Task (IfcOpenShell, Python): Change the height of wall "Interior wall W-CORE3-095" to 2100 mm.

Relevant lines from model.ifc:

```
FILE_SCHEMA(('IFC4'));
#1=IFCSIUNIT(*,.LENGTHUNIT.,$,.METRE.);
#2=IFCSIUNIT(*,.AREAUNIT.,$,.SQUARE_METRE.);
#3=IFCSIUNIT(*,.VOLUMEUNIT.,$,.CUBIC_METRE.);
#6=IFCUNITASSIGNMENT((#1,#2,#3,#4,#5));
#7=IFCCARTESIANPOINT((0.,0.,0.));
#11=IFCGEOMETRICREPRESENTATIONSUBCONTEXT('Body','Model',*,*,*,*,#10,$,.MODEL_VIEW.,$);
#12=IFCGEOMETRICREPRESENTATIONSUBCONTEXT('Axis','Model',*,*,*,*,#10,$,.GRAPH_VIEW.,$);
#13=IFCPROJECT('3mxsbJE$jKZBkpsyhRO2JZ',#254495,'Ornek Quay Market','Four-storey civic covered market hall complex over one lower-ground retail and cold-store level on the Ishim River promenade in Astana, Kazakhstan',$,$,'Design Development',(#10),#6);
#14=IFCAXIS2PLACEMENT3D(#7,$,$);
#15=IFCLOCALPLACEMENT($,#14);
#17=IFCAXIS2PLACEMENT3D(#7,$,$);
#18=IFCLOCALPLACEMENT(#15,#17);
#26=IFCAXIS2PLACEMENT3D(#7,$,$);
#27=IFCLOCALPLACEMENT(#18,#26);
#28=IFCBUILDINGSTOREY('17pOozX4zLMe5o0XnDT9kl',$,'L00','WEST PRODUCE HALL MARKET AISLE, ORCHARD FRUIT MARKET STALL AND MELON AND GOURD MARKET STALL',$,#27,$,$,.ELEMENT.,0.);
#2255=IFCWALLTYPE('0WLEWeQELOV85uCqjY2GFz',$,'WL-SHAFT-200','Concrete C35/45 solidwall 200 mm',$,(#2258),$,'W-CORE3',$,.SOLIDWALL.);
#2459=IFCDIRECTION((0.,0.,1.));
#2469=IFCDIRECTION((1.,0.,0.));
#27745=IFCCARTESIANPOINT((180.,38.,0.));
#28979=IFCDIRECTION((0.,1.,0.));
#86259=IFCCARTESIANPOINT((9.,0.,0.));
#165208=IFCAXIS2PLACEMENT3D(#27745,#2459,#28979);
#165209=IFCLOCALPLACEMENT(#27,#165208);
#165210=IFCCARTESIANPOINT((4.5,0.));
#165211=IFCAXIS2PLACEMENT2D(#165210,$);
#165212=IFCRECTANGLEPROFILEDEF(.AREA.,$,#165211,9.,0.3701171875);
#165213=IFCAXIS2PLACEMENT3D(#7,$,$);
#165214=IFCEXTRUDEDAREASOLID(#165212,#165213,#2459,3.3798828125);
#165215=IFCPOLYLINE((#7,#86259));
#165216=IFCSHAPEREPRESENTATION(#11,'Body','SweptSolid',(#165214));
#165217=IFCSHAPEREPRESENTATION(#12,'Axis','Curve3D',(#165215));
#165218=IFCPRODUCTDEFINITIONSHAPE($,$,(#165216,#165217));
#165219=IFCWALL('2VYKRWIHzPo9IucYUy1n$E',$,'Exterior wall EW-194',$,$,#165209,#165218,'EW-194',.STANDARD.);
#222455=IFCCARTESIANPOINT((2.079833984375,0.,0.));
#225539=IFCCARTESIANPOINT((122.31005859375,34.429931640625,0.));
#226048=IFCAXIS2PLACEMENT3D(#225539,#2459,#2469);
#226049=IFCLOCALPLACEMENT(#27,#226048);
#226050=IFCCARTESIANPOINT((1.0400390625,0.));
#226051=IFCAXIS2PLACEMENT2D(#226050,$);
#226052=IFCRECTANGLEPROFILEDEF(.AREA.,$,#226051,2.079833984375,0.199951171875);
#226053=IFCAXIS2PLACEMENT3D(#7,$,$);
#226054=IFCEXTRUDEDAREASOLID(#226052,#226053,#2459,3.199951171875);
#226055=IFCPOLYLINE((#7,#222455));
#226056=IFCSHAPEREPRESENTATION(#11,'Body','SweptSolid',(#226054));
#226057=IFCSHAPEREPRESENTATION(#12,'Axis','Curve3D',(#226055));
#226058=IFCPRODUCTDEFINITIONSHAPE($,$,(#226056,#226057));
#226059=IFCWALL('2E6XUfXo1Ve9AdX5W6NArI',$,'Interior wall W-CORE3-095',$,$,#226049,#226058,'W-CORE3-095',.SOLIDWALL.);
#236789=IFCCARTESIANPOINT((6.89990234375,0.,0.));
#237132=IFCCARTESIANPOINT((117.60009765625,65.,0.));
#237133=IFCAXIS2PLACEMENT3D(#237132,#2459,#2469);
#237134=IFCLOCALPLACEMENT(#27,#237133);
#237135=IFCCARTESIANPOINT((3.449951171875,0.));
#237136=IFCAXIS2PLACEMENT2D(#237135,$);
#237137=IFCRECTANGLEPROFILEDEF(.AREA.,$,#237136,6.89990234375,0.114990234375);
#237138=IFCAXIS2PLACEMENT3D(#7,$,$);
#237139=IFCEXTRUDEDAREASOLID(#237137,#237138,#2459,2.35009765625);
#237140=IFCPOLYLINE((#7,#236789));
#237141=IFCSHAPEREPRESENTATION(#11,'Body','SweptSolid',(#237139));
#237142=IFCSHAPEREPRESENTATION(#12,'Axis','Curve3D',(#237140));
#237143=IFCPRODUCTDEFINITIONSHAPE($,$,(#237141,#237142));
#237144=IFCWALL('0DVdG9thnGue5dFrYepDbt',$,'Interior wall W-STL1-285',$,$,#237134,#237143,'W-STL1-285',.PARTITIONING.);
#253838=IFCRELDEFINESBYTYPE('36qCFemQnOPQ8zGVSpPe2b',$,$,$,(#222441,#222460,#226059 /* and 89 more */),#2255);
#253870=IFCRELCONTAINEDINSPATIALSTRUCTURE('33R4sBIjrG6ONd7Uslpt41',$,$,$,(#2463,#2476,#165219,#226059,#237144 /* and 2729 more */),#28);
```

```python
import ifcopenshell
import ifcopenshell.geom
import ifcopenshell.util.representation
import ifcopenshell.util.shape

model = ifcopenshell.open("model.ifc")
settings = ifcopenshell.geom.settings()


def volume(element):
    """Net volume in cubic metres, openings subtracted."""
    shape = ifcopenshell.geom.create_shape(settings, element)
    return ifcopenshell.util.shape.get_volume(shape.geometry)


wall = model.by_guid("2E6XUfXo1Ve9AdX5W6NArI")
before = volume(wall)

body = ifcopenshell.util.representation.get_representation(wall, "Model", "Body")
solid = body.Items[0]
old_height = solid.Depth
solid.Depth = 2.1
after = volume(wall)

print(f"height {old_height:g} -> {solid.Depth:g}, volume {before:.3f} -> {after:.3f} m3")

model.write("model_rev.ifc")
```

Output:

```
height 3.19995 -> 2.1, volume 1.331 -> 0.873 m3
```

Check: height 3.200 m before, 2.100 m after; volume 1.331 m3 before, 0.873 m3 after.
